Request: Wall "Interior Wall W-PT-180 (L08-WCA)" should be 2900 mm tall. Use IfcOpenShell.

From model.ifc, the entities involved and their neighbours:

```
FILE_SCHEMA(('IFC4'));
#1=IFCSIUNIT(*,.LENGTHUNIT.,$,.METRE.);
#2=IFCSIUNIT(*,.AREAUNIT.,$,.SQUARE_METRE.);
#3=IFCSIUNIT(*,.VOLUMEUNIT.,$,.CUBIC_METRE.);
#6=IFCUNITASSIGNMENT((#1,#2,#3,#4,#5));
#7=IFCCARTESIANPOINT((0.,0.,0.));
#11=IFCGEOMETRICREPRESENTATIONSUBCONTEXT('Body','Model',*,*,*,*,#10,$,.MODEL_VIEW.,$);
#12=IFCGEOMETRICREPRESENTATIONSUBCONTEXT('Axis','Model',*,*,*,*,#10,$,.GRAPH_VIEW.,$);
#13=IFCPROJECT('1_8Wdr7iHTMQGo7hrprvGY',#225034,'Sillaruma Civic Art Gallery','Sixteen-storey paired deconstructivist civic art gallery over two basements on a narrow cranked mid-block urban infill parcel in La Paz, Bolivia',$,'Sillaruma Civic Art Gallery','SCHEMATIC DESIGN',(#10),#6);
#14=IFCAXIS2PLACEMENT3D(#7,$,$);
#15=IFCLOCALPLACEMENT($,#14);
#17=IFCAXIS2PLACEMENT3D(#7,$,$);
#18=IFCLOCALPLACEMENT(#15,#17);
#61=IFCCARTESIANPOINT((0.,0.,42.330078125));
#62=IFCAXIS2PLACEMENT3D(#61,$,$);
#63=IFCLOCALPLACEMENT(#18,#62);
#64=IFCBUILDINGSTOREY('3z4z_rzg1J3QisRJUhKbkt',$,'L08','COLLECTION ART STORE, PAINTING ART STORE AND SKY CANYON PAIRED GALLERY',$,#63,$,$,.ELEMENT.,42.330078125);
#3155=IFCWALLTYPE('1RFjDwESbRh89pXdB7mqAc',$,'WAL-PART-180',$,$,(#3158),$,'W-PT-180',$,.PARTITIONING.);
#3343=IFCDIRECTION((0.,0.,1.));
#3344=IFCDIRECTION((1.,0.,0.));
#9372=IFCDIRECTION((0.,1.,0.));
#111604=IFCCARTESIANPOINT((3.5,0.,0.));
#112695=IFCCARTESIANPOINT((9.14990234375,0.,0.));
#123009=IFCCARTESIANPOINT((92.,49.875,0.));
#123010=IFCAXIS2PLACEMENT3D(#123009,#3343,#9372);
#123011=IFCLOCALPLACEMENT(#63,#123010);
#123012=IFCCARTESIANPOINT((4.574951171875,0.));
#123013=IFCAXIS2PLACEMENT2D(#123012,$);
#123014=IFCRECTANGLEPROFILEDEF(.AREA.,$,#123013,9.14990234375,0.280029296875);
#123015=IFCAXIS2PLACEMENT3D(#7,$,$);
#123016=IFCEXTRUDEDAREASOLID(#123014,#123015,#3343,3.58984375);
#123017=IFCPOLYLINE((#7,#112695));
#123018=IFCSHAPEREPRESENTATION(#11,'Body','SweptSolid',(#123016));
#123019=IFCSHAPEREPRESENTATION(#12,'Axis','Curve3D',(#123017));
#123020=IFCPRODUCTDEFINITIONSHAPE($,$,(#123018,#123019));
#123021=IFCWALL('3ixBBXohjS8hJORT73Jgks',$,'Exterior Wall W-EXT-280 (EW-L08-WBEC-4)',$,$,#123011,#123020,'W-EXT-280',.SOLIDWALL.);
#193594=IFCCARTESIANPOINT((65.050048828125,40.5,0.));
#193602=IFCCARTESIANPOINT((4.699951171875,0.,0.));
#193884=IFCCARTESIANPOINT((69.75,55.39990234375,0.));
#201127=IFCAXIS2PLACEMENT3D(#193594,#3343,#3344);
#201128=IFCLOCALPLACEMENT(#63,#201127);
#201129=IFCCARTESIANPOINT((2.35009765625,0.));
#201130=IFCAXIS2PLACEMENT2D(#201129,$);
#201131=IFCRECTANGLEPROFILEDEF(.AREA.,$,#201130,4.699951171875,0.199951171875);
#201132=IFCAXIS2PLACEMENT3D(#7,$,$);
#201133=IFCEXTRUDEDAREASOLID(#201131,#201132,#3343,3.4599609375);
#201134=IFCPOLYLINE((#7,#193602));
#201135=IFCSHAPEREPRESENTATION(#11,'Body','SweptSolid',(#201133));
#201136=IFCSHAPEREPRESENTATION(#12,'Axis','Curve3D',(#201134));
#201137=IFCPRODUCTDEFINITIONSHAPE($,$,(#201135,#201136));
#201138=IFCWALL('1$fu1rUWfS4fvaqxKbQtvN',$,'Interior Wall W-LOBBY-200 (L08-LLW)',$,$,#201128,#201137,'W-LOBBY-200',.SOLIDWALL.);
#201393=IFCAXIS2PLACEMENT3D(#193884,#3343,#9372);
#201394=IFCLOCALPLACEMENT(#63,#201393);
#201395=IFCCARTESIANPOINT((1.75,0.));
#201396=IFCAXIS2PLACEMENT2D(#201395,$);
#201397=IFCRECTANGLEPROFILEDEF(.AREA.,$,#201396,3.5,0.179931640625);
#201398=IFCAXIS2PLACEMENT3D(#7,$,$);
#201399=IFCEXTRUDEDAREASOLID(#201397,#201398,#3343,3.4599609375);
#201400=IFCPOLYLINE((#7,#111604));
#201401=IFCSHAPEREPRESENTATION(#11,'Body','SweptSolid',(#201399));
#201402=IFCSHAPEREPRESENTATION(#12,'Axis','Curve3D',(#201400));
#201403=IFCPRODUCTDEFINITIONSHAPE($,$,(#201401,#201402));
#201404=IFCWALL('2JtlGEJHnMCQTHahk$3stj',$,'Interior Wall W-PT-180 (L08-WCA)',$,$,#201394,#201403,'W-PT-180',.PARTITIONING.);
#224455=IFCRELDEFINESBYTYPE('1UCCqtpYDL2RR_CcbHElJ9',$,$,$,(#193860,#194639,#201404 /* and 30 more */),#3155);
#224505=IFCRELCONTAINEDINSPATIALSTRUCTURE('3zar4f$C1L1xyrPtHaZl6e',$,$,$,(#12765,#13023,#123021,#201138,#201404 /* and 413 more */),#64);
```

```python
import ifcopenshell
import ifcopenshell.geom
import ifcopenshell.util.representation
import ifcopenshell.util.shape

model = ifcopenshell.open("model.ifc")
settings = ifcopenshell.geom.settings()


def volume(element):
    """Net volume in cubic metres, openings subtracted."""
    shape = ifcopenshell.geom.create_shape(settings, element)
    return ifcopenshell.util.shape.get_volume(shape.geometry)


wall = model.by_guid("2JtlGEJHnMCQTHahk$3stj")
before = volume(wall)

body = ifcopenshell.util.representation.get_representation(wall, "Model", "Body")
solid = body.Items[0]
old_height = solid.Depth
solid.Depth = 2.9
after = volume(wall)

print(f"height {old_height:g} -> {solid.Depth:g}, volume {before:.3f} -> {after:.3f} m3")

model.write("model_updated.ifc")
```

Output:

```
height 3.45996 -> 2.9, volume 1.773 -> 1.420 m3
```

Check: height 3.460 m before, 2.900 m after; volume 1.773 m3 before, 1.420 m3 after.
